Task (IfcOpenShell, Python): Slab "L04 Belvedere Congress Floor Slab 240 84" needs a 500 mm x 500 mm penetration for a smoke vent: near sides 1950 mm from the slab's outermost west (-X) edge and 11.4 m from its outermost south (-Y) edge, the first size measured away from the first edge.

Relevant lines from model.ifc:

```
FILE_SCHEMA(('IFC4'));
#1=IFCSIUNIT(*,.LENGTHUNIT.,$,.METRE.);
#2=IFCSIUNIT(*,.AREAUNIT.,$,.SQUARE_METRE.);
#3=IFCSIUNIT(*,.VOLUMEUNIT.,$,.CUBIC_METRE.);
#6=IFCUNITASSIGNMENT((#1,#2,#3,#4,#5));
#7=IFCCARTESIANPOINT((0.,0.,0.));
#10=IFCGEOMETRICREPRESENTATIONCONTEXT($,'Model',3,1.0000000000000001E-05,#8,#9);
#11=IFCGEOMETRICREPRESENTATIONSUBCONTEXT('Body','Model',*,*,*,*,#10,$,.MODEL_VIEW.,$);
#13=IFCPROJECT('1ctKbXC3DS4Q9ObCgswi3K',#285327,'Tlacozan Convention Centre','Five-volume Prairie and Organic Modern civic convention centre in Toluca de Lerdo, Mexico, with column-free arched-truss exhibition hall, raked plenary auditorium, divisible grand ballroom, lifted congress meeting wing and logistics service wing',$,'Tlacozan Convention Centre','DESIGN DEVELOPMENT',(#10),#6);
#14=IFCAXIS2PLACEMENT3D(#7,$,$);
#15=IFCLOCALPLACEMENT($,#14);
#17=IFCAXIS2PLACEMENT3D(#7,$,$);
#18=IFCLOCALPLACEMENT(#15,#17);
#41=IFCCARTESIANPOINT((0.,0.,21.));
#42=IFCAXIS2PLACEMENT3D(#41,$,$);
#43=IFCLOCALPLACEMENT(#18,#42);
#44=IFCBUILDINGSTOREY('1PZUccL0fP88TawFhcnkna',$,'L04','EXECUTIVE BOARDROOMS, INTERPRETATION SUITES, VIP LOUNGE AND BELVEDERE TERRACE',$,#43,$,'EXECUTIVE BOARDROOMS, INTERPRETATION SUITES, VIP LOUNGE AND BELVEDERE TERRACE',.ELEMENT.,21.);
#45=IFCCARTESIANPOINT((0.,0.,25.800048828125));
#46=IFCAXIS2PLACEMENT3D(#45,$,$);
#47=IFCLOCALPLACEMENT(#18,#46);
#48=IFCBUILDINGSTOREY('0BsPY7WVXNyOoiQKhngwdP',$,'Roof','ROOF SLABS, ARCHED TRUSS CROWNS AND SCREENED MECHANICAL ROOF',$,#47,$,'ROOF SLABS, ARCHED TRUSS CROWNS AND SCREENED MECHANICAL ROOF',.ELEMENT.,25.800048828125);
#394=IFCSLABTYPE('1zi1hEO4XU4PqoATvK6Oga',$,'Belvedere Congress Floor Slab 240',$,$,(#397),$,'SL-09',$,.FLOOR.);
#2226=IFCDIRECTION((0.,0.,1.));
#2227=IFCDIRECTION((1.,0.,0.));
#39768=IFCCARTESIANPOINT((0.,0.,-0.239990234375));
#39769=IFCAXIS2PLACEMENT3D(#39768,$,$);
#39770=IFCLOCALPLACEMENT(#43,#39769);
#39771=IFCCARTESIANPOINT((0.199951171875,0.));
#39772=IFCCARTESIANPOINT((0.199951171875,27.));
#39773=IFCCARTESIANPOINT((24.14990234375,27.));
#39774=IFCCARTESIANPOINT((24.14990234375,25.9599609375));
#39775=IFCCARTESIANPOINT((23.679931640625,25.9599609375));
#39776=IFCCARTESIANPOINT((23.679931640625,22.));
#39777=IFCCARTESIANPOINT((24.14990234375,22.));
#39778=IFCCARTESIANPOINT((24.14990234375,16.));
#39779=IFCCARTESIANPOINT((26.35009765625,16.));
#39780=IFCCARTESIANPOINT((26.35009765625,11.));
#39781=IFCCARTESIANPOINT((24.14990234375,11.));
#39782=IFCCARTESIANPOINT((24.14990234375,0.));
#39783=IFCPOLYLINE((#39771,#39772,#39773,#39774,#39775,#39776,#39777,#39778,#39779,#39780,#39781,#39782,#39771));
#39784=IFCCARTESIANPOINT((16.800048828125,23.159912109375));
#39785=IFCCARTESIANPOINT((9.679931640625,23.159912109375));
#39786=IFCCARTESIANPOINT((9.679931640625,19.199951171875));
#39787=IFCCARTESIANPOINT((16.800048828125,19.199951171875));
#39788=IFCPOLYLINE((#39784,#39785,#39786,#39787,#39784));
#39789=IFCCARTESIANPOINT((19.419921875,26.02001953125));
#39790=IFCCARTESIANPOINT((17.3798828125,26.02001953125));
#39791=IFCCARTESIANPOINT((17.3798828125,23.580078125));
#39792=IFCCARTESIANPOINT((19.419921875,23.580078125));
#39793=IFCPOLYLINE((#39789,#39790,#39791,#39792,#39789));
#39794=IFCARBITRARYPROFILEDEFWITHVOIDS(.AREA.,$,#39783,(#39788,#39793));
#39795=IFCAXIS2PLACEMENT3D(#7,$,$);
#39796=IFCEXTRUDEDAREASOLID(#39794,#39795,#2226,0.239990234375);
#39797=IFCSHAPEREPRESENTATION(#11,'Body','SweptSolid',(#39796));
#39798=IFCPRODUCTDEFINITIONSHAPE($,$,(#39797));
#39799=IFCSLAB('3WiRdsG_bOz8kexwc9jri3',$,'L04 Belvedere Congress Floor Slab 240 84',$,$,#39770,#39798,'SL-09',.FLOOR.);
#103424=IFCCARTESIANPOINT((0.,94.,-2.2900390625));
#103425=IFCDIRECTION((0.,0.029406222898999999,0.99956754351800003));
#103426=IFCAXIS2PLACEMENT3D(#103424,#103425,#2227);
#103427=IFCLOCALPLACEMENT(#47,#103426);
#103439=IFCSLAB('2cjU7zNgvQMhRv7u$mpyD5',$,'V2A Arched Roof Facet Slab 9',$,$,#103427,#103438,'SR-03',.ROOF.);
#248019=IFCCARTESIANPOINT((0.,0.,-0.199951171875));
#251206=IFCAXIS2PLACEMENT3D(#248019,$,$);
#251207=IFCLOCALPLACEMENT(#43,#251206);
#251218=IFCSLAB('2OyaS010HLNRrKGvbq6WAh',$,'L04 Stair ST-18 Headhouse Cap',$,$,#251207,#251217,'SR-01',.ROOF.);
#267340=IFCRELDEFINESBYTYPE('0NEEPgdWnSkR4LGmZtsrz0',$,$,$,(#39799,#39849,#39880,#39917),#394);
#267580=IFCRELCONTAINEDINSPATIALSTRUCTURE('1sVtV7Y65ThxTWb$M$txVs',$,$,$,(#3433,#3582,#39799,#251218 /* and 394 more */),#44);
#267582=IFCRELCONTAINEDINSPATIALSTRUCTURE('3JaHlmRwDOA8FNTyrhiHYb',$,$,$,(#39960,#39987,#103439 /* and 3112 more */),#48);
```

```python
import numpy as np
import ifcopenshell
import ifcopenshell.api.feature
import ifcopenshell.api.geometry
import ifcopenshell.api.root
import ifcopenshell.geom
import ifcopenshell.util.placement
import ifcopenshell.util.representation
import ifcopenshell.util.shape
import ifcopenshell.util.unit

model = ifcopenshell.open("model.ifc")
unit_scale = ifcopenshell.util.unit.calculate_unit_scale(model)
settings = ifcopenshell.geom.settings()


def volume(element):
    """Net volume in cubic metres, openings subtracted."""
    shape = ifcopenshell.geom.create_shape(settings, element)
    return ifcopenshell.util.shape.get_volume(shape.geometry)


slab = model.by_guid("3WiRdsG_bOz8kexwc9jri3")
before = volume(slab)

# Extent in the slab's own axes, in metres. The edges named are its -X and -Y sides.
slab_shape = ifcopenshell.geom.create_shape(settings, slab)
vertices = ifcopenshell.util.shape.get_vertices(slab_shape.geometry)
x_min, y_min, bottom = vertices.min(axis=0)
top = vertices[:, 2].max()

opening = ifcopenshell.api.root.create_entity(model, ifc_class="IfcOpeningElement", name="Smoke vent opening", predefined_type="OPENING")
context = ifcopenshell.util.representation.get_context(model, "Model", "Body", "MODEL_VIEW")
width, depth = 0.5, 0.5
outline = [(0.0, 0.0), (width, 0.0), (width, depth), (0.0, depth), (0.0, 0.0)]
# Overshoot both faces by 50 mm so the cut is clean.
shape = ifcopenshell.api.geometry.add_slab_representation(
    model, context=context, depth=top - bottom + 0.1, polyline=outline
)
ifcopenshell.api.geometry.assign_representation(model, product=opening, representation=shape)

matrix = ifcopenshell.util.placement.get_local_placement(slab.ObjectPlacement)
matrix[:, 3] = matrix @ np.append(np.array([x_min + 1.95, y_min + 11.4, bottom - 0.05]) / unit_scale, 1.0)
ifcopenshell.api.geometry.edit_object_placement(model, product=opening, matrix=matrix, is_si=False)
ifcopenshell.api.feature.add_feature(model, feature=opening, element=slab)

after = volume(slab)

print(f"slab volume {before:.3f} -> {after:.3f} m3")

model.write("model-out.ifc")
```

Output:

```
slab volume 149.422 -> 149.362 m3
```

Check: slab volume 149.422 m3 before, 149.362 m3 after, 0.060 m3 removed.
